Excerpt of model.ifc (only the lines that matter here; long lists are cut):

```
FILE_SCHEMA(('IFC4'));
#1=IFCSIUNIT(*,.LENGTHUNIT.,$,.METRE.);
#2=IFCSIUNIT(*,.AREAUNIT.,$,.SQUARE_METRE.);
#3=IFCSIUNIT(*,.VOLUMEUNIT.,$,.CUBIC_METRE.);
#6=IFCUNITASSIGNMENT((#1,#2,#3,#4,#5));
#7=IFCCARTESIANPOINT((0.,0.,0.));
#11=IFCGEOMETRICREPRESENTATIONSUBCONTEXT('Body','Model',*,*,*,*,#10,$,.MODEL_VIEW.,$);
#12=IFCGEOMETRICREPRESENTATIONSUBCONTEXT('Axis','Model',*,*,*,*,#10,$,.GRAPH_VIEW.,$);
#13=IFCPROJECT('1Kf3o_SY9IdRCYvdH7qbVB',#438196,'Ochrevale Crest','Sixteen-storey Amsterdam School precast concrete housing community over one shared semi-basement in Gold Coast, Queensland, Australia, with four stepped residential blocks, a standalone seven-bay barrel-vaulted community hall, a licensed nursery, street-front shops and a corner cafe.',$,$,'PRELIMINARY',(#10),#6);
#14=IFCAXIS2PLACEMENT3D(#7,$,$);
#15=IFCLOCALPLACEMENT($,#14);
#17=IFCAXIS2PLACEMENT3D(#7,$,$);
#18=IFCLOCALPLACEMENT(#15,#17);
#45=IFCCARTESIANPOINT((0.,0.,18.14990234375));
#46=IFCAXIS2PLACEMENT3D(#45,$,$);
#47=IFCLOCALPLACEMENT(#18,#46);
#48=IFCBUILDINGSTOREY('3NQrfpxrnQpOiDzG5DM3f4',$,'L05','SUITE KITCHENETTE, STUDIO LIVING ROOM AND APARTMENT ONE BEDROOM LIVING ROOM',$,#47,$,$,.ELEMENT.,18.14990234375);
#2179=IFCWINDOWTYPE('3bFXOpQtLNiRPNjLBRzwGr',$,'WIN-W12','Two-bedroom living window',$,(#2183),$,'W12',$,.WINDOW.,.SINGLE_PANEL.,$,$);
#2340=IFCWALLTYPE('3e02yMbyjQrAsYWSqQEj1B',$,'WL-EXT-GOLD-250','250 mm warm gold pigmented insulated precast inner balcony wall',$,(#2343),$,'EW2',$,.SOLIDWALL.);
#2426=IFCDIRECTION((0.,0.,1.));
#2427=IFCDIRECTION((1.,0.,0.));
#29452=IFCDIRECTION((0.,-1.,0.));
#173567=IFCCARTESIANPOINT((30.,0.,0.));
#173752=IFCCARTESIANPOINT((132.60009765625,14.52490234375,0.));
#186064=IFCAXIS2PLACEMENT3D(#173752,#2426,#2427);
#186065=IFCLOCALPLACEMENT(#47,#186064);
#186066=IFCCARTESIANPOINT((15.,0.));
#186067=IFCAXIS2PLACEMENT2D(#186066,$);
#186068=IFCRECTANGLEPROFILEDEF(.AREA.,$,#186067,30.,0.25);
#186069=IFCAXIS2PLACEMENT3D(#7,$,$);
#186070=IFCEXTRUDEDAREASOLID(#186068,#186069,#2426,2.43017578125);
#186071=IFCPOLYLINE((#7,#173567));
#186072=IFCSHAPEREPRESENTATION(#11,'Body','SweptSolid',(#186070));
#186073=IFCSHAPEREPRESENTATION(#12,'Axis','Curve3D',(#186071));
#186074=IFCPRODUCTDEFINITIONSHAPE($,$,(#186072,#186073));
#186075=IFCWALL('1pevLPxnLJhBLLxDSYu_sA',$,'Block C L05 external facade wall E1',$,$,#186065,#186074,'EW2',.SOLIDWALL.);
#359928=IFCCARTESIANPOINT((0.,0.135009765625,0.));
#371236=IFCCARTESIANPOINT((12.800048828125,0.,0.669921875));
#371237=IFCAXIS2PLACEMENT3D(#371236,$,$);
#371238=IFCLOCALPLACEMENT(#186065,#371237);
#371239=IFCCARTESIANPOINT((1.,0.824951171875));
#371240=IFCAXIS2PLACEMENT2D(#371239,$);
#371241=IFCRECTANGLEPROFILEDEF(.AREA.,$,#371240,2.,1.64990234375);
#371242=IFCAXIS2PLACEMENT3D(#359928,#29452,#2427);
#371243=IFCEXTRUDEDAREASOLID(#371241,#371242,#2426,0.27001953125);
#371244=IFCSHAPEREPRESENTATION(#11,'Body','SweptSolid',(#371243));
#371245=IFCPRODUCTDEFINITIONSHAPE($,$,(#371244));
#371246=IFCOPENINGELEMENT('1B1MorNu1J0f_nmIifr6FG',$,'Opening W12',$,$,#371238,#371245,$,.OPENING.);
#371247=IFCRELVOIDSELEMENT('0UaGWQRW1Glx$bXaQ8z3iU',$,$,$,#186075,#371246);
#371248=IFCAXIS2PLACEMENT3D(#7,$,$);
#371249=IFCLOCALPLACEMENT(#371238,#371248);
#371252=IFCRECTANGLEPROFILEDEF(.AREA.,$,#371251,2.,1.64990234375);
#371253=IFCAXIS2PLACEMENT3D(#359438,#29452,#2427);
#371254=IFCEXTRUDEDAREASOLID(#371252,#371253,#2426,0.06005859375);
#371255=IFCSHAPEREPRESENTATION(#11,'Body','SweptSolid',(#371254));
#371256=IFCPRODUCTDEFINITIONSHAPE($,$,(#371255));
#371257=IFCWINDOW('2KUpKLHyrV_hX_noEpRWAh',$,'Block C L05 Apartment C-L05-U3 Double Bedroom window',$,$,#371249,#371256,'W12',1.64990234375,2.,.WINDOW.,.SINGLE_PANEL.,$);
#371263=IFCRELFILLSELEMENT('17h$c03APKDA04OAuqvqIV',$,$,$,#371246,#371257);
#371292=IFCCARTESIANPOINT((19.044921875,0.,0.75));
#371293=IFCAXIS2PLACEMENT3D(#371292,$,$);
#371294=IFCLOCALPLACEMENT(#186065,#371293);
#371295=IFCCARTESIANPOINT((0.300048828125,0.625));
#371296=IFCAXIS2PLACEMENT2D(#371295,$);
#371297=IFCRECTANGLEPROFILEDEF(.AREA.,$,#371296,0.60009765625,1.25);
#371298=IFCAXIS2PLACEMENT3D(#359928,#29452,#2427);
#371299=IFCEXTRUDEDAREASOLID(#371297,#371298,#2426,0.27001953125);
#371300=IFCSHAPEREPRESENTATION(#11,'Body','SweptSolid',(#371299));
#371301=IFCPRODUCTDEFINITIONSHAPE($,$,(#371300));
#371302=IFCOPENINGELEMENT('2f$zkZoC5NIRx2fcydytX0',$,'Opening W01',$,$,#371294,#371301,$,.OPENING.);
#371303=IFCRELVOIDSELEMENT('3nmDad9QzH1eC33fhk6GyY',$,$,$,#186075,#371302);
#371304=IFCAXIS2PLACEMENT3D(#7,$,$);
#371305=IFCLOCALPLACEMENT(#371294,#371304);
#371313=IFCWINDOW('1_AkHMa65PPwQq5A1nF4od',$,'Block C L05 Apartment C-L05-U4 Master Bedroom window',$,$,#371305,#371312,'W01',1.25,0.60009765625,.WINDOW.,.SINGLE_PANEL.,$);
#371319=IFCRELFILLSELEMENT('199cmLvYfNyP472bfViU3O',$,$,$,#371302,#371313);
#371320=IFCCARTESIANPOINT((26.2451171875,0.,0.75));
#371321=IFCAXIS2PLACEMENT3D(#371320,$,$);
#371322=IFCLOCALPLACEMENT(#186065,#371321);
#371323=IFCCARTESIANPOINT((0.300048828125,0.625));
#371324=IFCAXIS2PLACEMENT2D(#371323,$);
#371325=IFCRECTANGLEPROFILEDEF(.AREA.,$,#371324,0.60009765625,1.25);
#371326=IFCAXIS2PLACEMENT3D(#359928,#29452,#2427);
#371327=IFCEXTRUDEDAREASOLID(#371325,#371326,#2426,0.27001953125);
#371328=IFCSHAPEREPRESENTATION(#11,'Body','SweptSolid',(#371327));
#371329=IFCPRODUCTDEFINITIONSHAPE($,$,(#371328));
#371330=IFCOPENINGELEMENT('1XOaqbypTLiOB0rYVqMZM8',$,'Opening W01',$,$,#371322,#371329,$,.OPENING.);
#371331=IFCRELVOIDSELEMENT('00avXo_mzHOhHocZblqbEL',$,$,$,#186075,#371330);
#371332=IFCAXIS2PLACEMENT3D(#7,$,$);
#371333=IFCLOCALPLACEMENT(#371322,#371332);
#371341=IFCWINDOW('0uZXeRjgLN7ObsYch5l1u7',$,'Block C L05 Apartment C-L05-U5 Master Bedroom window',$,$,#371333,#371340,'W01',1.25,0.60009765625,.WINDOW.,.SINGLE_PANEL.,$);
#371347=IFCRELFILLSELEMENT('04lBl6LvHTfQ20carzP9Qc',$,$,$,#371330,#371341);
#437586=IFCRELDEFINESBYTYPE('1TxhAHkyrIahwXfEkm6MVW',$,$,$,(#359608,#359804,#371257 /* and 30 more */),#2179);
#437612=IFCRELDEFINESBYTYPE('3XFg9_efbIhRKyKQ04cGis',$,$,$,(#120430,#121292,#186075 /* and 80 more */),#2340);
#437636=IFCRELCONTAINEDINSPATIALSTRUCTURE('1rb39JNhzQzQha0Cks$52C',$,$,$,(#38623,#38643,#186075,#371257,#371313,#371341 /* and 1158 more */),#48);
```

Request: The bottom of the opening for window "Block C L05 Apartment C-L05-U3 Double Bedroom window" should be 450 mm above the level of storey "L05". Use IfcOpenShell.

```python
import numpy as np
import ifcopenshell
import ifcopenshell.api.geometry
import ifcopenshell.geom
import ifcopenshell.util.element
import ifcopenshell.util.placement
import ifcopenshell.util.shape
import ifcopenshell.util.unit

model = ifcopenshell.open("model.ifc")
unit_scale = ifcopenshell.util.unit.calculate_unit_scale(model)

window = model.by_id(371257)
opening = window.FillsVoids[0].RelatingOpeningElement
storey = ifcopenshell.util.element.get_container(window, ifc_class="IfcBuildingStorey")
level = ifcopenshell.util.placement.get_local_placement(storey.ObjectPlacement)[2, 3]

# The opening's origin need not be at the sill, so measure its lowest point.
shape = ifcopenshell.geom.create_shape(ifcopenshell.geom.settings(), opening)
bottom = ifcopenshell.util.shape.get_shape_bottom_elevation(shape, shape.geometry) / unit_scale
dz = level + 0.45 / unit_scale - bottom

shift = np.array([0.0, 0.0, dz])
# The window is placed relative to its opening, so it follows when the opening moves.
matrix = ifcopenshell.util.placement.get_local_placement(opening.ObjectPlacement)
matrix[:3, 3] += shift
ifcopenshell.api.geometry.edit_object_placement(
    model, product=opening, matrix=matrix, is_si=False, should_transform_children=True
)

print(f"moved by {dz * unit_scale:+.3f} m")

model.write("model_updated.ifc")
```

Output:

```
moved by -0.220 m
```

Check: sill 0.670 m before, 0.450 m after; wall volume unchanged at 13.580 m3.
